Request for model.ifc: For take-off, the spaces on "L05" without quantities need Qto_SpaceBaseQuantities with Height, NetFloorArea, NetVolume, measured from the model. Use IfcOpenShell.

First a look at what the model holds.

```python
import ifcopenshell
import ifcopenshell.util.element
import ifcopenshell.util.unit

model = ifcopenshell.open("model.ifc")
print(model.schema)
for unit_type in ("LENGTHUNIT", "AREAUNIT", "VOLUMEUNIT"):
    print(unit_type, ifcopenshell.util.unit.calculate_unit_scale(model, unit_type))
storey = next(s for s in model.by_type("IfcBuildingStorey") if s.Name == "L05")
spaces = [e for e in ifcopenshell.util.element.get_decomposition(storey) if e.is_a("IfcSpace")]
for e in sorted(spaces, key=lambda e: e.id()):
    print(e.id(), e.is_a(), e.Name, list(ifcopenshell.util.element.get_psets(e, qtos_only=True)), sep=" | ")
```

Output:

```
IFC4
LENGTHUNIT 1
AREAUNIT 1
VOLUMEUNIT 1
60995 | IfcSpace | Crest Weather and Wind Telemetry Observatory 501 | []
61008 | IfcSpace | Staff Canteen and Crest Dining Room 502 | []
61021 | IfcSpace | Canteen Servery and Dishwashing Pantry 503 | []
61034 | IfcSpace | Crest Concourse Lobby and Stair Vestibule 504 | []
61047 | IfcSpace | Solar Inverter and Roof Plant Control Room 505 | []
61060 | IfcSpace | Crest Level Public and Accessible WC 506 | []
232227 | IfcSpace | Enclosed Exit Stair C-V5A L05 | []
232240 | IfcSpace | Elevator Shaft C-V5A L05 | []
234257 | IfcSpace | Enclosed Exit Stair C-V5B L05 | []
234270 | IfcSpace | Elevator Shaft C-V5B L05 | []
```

```python
import ifcopenshell
import ifcopenshell.api.pset
import ifcopenshell.geom
import ifcopenshell.util.element
import ifcopenshell.util.shape
import ifcopenshell.util.unit

model = ifcopenshell.open("model.ifc")
unit_scale = ifcopenshell.util.unit.calculate_unit_scale(model)
area_scale = ifcopenshell.util.unit.calculate_unit_scale(model, "AREAUNIT")
volume_scale = ifcopenshell.util.unit.calculate_unit_scale(model, "VOLUMEUNIT")
settings = ifcopenshell.geom.settings()

storey = next(s for s in model.by_type("IfcBuildingStorey") if s.Name == "L05")
spaces = [e for e in ifcopenshell.util.element.get_decomposition(storey) if e.is_a("IfcSpace")]

for e in sorted(spaces, key=lambda e: e.id()):
    if ifcopenshell.util.element.get_psets(e, qtos_only=True, should_inherit=False):
        continue
    # Geometry comes back in metres, in the element's own axes.
    shape = ifcopenshell.geom.create_shape(settings, e)
    values = {
        "Height": ifcopenshell.util.shape.get_z(shape.geometry) / unit_scale,
        "NetFloorArea": ifcopenshell.util.shape.get_footprint_area(shape.geometry) / area_scale,
        "NetVolume": ifcopenshell.util.shape.get_volume(shape.geometry) / volume_scale,
    }
    qto = ifcopenshell.api.pset.add_qto(model, product=e, name="Qto_SpaceBaseQuantities")
    ifcopenshell.api.pset.edit_qto(model, qto=qto, properties=values)
    print(e.id(), {k: round(v, 3) for k, v in values.items()})

model.write("model-out.ifc")
```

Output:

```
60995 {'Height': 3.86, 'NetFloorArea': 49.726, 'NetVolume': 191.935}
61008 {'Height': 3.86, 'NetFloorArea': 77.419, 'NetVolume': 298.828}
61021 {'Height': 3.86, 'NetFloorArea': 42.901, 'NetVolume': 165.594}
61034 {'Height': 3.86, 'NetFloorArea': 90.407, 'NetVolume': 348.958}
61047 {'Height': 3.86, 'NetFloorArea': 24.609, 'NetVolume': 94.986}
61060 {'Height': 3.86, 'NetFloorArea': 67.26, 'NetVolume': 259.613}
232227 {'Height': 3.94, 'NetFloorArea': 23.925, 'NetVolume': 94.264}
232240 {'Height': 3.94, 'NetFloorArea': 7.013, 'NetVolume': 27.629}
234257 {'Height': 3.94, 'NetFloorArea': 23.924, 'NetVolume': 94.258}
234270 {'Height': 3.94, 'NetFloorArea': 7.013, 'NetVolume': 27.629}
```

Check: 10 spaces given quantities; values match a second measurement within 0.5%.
